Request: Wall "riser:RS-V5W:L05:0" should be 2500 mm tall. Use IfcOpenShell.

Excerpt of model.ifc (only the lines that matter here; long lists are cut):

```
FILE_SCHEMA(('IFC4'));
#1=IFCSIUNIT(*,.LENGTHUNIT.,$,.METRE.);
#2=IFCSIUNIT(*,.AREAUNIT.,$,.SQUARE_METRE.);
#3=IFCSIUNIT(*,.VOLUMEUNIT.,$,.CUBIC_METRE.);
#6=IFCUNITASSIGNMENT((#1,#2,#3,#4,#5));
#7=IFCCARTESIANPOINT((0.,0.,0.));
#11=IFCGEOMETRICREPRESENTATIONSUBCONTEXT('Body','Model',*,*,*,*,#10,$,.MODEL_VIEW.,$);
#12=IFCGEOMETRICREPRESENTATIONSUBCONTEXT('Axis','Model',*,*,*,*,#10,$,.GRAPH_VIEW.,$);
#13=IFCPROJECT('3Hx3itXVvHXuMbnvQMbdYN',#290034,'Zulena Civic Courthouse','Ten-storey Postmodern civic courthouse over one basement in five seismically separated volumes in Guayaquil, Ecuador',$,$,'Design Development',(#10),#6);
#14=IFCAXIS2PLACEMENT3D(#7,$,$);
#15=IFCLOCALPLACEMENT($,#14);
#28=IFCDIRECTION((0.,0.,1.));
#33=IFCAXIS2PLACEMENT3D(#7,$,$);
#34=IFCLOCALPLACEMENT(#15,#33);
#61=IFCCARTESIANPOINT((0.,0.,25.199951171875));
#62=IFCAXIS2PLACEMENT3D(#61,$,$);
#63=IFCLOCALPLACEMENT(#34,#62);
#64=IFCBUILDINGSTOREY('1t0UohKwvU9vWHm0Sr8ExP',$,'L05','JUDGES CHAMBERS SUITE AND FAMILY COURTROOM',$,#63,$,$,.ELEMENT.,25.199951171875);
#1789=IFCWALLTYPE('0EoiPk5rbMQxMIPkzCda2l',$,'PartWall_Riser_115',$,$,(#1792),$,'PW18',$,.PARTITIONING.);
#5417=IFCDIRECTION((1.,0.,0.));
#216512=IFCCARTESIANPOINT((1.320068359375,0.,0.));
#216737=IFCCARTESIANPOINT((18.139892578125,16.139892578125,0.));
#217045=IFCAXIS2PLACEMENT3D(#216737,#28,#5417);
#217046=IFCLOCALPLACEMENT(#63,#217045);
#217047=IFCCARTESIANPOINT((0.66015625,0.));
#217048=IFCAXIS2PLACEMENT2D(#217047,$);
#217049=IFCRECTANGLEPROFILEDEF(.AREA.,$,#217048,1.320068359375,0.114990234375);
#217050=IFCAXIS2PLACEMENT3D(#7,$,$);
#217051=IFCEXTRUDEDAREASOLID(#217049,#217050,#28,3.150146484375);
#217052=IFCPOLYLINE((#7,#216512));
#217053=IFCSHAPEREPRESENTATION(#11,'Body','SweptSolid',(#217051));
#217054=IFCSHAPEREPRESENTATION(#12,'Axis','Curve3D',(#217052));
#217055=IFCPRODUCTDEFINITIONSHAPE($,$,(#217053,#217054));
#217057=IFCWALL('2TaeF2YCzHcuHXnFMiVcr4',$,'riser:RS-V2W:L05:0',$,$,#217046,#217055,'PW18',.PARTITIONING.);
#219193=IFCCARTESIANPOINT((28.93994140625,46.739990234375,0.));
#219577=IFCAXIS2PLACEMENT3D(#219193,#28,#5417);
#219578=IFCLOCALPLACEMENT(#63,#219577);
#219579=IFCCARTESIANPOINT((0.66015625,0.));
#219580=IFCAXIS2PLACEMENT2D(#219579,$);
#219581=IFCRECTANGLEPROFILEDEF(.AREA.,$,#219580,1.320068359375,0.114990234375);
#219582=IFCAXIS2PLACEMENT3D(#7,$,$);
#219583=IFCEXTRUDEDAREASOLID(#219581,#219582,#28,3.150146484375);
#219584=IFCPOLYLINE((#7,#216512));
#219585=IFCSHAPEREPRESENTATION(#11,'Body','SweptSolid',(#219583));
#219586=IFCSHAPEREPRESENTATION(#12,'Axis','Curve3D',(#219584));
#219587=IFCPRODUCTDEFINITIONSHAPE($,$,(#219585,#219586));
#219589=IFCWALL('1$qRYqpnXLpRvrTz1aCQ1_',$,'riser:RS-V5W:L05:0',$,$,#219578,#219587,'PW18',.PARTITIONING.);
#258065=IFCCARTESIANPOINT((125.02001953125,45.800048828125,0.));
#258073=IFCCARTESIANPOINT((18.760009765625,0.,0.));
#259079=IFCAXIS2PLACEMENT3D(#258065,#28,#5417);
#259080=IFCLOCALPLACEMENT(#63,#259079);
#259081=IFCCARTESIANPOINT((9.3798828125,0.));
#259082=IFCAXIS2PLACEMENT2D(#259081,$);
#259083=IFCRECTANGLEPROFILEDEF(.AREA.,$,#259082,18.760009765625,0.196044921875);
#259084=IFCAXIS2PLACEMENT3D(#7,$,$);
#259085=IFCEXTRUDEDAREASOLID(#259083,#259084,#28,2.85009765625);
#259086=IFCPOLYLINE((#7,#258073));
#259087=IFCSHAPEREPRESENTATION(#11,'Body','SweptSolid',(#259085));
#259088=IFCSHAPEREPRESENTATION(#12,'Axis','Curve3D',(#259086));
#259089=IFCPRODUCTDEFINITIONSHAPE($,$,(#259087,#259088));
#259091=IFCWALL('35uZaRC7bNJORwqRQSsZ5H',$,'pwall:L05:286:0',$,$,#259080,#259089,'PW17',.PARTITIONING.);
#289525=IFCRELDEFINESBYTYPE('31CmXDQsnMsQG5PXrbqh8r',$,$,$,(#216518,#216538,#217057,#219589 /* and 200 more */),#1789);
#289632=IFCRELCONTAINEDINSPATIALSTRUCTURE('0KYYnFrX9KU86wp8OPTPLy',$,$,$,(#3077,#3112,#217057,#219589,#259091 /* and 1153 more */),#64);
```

```python
import ifcopenshell
import ifcopenshell.geom
import ifcopenshell.util.representation
import ifcopenshell.util.shape
import ifcopenshell.util.unit

model = ifcopenshell.open("model.ifc")
unit_scale = ifcopenshell.util.unit.calculate_unit_scale(model)
settings = ifcopenshell.geom.settings()


def volume(element):
    """Net volume in cubic metres, openings subtracted."""
    shape = ifcopenshell.geom.create_shape(settings, element)
    return ifcopenshell.util.shape.get_volume(shape.geometry)


wall = model.by_id(219589)
before = volume(wall)

body = ifcopenshell.util.representation.get_representation(wall, "Model", "Body")
solid = body.Items[0]
old_height = solid.Depth
solid.Depth = 2.5 / unit_scale
after = volume(wall)

print(f"height {old_height:g} -> {solid.Depth:g}, volume {before:.3f} -> {after:.3f} m3")

model.write("model_v2.ifc")
```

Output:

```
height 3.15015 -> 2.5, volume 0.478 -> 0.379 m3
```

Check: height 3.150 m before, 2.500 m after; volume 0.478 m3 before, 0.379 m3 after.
